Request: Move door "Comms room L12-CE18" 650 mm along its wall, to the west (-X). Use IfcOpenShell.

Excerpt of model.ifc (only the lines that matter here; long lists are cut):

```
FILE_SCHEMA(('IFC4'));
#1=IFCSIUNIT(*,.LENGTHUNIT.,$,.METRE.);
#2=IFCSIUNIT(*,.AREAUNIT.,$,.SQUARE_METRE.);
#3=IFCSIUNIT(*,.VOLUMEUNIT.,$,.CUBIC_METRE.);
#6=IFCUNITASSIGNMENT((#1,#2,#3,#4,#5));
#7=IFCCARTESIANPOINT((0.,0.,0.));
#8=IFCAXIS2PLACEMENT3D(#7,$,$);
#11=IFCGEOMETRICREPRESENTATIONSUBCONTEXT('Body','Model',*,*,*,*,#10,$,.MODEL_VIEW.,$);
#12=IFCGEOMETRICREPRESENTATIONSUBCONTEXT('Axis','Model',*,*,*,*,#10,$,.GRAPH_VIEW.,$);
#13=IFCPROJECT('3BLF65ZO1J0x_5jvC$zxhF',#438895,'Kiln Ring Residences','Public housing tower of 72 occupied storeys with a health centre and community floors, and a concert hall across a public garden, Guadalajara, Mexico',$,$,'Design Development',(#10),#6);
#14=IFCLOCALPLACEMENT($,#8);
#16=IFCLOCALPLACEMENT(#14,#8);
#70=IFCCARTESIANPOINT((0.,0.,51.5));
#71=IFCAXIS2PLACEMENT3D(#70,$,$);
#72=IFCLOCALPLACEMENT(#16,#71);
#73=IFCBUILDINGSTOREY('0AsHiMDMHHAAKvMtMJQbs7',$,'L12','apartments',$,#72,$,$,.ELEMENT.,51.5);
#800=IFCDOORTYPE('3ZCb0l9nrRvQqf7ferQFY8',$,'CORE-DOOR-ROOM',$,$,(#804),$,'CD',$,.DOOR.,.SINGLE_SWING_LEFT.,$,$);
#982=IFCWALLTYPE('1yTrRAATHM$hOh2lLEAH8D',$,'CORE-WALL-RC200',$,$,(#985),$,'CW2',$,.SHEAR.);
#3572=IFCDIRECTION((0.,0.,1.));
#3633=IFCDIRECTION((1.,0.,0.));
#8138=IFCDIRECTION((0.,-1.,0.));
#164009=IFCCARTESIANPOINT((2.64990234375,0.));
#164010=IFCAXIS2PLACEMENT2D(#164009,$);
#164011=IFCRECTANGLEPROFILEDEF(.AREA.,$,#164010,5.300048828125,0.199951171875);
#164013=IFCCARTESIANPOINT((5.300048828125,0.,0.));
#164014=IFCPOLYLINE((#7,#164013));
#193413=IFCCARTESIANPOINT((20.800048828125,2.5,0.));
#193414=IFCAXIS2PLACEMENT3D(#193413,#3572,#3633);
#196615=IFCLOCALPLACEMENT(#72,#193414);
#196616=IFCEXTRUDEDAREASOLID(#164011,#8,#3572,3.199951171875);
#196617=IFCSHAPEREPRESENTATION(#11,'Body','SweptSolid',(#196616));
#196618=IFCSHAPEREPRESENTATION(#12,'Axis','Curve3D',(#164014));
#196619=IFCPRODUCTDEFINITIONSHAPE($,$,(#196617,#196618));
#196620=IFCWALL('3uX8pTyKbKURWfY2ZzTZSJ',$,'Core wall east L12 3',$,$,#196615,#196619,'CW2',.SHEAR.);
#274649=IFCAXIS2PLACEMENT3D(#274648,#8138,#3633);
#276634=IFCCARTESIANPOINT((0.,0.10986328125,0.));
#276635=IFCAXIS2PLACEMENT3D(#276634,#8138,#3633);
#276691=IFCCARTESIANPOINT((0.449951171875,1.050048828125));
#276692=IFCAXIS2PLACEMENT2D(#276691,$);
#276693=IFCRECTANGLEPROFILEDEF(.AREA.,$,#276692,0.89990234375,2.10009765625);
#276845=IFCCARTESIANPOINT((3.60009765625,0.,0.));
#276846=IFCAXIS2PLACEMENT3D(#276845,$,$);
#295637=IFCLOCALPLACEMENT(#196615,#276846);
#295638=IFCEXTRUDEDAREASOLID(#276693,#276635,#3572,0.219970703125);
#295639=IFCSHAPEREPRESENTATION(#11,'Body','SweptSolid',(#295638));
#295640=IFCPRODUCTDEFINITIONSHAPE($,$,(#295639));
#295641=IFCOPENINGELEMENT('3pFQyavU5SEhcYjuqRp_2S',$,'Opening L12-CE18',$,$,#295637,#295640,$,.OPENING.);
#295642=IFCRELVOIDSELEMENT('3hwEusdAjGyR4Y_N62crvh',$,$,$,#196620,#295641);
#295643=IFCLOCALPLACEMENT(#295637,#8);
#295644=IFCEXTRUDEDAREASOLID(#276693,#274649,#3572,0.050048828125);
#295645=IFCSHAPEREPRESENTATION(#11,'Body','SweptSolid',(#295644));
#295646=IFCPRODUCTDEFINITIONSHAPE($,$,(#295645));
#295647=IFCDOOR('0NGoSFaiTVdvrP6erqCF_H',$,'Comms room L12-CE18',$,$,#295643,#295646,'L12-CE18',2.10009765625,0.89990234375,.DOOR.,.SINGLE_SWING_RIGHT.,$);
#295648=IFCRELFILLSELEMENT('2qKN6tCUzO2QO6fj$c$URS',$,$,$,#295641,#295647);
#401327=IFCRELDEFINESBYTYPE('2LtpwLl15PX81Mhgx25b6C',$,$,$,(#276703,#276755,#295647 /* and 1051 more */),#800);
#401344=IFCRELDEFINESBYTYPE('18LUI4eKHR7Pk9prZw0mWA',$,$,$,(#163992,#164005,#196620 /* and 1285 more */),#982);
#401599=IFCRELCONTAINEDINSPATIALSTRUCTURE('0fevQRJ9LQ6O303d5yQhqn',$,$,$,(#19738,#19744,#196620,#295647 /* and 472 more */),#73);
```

```python
import ifcopenshell
import ifcopenshell.api.geometry
import ifcopenshell.util.placement
import ifcopenshell.util.unit

model = ifcopenshell.open("model.ifc")
unit_scale = ifcopenshell.util.unit.calculate_unit_scale(model)

door = model.by_id(295647)
opening = door.FillsVoids[0].RelatingOpeningElement
wall = opening.VoidsElements[0].RelatingBuildingElement

wall_matrix = ifcopenshell.util.placement.get_local_placement(wall.ObjectPlacement)
shift = wall_matrix[:3, 0] * -0.65 / unit_scale
before = ifcopenshell.util.placement.get_local_placement(door.ObjectPlacement)[:3, 3].copy()

# The door is placed relative to its opening, so it follows when the opening moves.
matrix = ifcopenshell.util.placement.get_local_placement(opening.ObjectPlacement)
matrix[:3, 3] += shift
ifcopenshell.api.geometry.edit_object_placement(
    model, product=opening, matrix=matrix, is_si=False, should_transform_children=True
)

after = ifcopenshell.util.placement.get_local_placement(door.ObjectPlacement)[:3, 3]
print("door moved by", (after - before).round(3) + 0.0)

model.write("model-out.ifc")
```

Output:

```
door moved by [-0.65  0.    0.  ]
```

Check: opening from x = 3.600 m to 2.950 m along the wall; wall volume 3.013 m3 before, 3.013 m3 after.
